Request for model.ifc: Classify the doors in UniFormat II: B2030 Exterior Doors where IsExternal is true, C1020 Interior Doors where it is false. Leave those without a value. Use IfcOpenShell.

First a look at what the model holds.

```python
import ifcopenshell
import ifcopenshell.util.element

model = ifcopenshell.open("model.ifc")
print(model.schema)
print("classifications:", [c.Name for c in model.by_type("IfcClassification")])
values = [ifcopenshell.util.element.get_pset(e, "Pset_DoorCommon", "IsExternal") for e in model.by_type("IfcDoor")]
for value in (True, False, None):
    print("IsExternal", value, values.count(value))
```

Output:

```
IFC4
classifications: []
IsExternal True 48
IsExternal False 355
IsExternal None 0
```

```python
import ifcopenshell
import ifcopenshell.api.classification
import ifcopenshell.util.element

model = ifcopenshell.open("model.ifc")

system = ifcopenshell.api.classification.add_classification(model, classification="UniFormat II")

doors = model.by_type("IfcDoor")
external = {e: ifcopenshell.util.element.get_pset(e, "Pset_DoorCommon", "IsExternal") for e in doors}
for flag, code, name in ((True, "B2030", "Exterior Doors"), (False, "C1020", "Interior Doors")):
    products = [e for e in doors if external[e] is flag]
    ifcopenshell.api.classification.add_reference(
        model, products=products, classification=system, identification=code, name=name
    )
    print(code, len(products))

model.write("model_edited.ifc")
```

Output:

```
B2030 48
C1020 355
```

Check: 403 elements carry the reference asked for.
